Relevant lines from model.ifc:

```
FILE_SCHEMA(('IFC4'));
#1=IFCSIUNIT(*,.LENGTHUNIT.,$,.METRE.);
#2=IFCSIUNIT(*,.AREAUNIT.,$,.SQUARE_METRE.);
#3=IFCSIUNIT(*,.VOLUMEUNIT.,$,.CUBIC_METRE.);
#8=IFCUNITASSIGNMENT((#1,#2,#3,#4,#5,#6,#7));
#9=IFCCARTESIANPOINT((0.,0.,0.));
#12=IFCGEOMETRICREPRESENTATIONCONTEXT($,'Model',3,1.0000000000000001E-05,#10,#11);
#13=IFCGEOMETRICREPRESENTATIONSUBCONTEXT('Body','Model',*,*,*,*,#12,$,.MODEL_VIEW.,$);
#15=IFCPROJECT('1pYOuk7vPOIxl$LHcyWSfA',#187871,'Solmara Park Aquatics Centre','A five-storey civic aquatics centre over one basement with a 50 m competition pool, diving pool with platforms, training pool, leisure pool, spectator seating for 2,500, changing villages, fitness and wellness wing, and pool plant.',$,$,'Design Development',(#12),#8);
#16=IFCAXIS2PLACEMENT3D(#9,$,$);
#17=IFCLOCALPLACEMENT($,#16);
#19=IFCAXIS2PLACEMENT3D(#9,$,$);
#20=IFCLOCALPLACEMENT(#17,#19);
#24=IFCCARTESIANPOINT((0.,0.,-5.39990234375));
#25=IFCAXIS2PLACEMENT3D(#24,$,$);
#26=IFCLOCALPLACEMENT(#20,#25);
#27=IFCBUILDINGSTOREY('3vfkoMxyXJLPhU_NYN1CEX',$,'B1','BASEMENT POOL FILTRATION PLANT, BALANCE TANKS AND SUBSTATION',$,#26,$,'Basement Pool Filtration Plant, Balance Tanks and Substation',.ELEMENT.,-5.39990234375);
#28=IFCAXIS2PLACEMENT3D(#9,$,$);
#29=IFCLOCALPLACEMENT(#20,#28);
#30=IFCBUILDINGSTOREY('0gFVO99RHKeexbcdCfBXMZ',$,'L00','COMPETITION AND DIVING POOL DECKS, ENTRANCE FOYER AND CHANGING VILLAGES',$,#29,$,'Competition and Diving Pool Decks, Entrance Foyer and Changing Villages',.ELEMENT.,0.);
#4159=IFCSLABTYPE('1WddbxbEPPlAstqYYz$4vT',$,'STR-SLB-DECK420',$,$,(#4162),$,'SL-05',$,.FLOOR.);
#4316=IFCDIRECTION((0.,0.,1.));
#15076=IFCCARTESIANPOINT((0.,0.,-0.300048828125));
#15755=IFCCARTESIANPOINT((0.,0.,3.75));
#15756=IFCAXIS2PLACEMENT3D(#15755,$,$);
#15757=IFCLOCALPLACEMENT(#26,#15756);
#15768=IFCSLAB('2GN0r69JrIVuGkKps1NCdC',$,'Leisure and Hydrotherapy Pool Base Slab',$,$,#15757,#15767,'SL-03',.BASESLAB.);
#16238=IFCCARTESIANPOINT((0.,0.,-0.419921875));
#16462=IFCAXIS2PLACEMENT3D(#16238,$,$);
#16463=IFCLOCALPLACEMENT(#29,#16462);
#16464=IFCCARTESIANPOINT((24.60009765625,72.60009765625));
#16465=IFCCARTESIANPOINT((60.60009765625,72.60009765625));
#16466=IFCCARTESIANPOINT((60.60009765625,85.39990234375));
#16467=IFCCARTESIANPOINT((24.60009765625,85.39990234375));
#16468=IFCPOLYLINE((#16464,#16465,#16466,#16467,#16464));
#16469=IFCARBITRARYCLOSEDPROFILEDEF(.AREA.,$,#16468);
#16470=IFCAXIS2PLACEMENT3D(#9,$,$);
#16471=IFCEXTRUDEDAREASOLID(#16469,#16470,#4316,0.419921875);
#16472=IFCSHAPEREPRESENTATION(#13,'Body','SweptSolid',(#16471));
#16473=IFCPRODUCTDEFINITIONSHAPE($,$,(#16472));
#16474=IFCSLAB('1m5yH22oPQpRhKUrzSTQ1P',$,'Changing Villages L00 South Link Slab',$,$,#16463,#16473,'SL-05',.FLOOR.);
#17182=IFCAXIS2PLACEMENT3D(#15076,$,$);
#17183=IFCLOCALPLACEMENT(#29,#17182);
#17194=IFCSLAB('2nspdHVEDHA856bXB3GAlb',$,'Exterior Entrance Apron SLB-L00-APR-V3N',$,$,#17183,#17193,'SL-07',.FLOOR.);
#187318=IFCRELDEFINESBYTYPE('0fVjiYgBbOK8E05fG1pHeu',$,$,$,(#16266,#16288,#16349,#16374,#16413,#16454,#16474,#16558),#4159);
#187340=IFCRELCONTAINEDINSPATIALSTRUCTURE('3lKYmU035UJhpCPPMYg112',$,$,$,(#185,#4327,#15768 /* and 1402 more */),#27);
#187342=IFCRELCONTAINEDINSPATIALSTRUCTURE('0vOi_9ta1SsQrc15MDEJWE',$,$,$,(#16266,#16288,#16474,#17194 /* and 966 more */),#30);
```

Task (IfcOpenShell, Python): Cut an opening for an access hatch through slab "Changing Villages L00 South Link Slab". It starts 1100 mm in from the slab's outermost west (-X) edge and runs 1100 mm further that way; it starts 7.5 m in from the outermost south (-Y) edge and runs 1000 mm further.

```python
import numpy as np
import ifcopenshell
import ifcopenshell.api.feature
import ifcopenshell.api.geometry
import ifcopenshell.api.root
import ifcopenshell.geom
import ifcopenshell.util.placement
import ifcopenshell.util.representation
import ifcopenshell.util.shape
import ifcopenshell.util.unit

model = ifcopenshell.open("model.ifc")
unit_scale = ifcopenshell.util.unit.calculate_unit_scale(model)
settings = ifcopenshell.geom.settings()


def volume(element):
    """Net volume in cubic metres, openings subtracted."""
    shape = ifcopenshell.geom.create_shape(settings, element)
    return ifcopenshell.util.shape.get_volume(shape.geometry)


slab = model.by_id(16474)
before = volume(slab)

# Extent in the slab's own axes, in metres. The edges named are its -X and -Y sides.
slab_shape = ifcopenshell.geom.create_shape(settings, slab)
vertices = ifcopenshell.util.shape.get_vertices(slab_shape.geometry)
x_min, y_min, bottom = vertices.min(axis=0)
top = vertices[:, 2].max()

opening = ifcopenshell.api.root.create_entity(model, ifc_class="IfcOpeningElement", name="Access hatch opening", predefined_type="OPENING")
context = ifcopenshell.util.representation.get_context(model, "Model", "Body", "MODEL_VIEW")
width, depth = 1.1, 1
outline = [(0.0, 0.0), (width, 0.0), (width, depth), (0.0, depth), (0.0, 0.0)]
# Overshoot both faces by 50 mm so the cut is clean.
shape = ifcopenshell.api.geometry.add_slab_representation(
    model, context=context, depth=top - bottom + 0.1, polyline=outline
)
ifcopenshell.api.geometry.assign_representation(model, product=opening, representation=shape)

matrix = ifcopenshell.util.placement.get_local_placement(slab.ObjectPlacement)
matrix[:, 3] = matrix @ np.append(np.array([x_min + 1.1, y_min + 7.5, bottom - 0.05]) / unit_scale, 1.0)
ifcopenshell.api.geometry.edit_object_placement(model, product=opening, matrix=matrix, is_si=False)
ifcopenshell.api.feature.add_feature(model, feature=opening, element=slab)

after = volume(slab)

print(f"slab volume {before:.3f} -> {after:.3f} m3")

model.write("model_updated.ifc")
```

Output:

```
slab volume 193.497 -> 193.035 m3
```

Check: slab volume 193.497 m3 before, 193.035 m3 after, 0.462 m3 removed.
